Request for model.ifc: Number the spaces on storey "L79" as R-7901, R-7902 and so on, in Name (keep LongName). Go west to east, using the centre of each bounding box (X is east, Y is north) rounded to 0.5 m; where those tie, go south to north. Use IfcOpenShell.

First a look at what the model holds.

```python
import ifcopenshell
import ifcopenshell.util.element
import ifcopenshell.util.placement

model = ifcopenshell.open("model.ifc")
print(model.schema)
storey = next(s for s in model.by_type("IfcBuildingStorey") if s.Name == "L79")
spaces = [e for e in ifcopenshell.util.element.get_decomposition(storey) if e.is_a("IfcSpace")]
for e in sorted(spaces, key=lambda e: e.id()):
    origin = ifcopenshell.util.placement.get_local_placement(e.ObjectPlacement)[:3, 3]
    print(e.id(), e.Name, e.LongName, origin.round(2) + 0.0, sep=" | ")
```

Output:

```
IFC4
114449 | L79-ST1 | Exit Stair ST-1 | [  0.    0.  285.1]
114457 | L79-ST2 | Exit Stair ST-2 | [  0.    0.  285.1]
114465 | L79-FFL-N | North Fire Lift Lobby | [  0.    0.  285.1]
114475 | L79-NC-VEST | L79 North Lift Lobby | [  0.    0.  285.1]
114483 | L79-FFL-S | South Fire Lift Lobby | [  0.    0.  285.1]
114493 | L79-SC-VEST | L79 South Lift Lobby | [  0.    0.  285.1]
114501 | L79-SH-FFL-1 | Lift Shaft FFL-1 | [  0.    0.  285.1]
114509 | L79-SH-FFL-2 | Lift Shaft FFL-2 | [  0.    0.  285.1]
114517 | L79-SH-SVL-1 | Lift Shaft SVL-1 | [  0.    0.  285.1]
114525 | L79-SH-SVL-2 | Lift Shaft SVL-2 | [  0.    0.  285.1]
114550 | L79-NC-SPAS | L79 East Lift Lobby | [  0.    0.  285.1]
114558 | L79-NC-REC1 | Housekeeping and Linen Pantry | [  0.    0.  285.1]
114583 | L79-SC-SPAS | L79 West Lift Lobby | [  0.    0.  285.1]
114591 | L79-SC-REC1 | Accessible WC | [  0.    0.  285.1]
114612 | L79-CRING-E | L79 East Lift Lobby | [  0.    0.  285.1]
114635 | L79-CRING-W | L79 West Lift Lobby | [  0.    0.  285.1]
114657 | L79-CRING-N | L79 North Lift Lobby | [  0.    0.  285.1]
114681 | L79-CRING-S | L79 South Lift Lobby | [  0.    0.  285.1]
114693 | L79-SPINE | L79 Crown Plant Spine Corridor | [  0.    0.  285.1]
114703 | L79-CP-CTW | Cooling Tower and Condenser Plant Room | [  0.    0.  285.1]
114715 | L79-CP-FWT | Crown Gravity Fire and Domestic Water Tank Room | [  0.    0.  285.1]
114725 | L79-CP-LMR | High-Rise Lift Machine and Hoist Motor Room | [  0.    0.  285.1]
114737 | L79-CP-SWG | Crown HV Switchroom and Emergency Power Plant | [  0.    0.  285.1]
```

```python
import ifcopenshell
import ifcopenshell.geom
import ifcopenshell.util.element
import ifcopenshell.util.shape

model = ifcopenshell.open("model.ifc")
settings = ifcopenshell.geom.settings()
settings.set("use-world-coords", True)


def centre(element):
    shape = ifcopenshell.geom.create_shape(settings, element)
    return ifcopenshell.util.shape.get_bbox_centroid(shape.geometry)


storey = next(s for s in model.by_type("IfcBuildingStorey") if s.Name == "L79")
spaces = [e for e in ifcopenshell.util.element.get_decomposition(storey) if e.is_a("IfcSpace")]

# Insertion points can sit at a corner or the storey origin, so sort by the geometry (in metres).
centres = {e: centre(e) for e in spaces}
spaces.sort(key=lambda e: (round(centres[e][0] / 0.5), centres[e][1]))

for i, e in enumerate(spaces, start=1):
    number = f"R-79{i:02d}"
    e.Name = number
    print(e.id(), number)

model.write("model_rev.ifc")
```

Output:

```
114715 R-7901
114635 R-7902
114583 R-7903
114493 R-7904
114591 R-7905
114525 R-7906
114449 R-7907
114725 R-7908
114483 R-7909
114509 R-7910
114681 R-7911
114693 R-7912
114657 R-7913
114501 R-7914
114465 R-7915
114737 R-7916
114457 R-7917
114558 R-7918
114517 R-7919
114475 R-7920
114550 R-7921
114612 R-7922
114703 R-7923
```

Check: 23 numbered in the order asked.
